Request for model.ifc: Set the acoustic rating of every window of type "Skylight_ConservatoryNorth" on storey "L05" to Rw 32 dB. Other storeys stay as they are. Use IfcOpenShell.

First a look at what the model holds.

```python
import ifcopenshell
import ifcopenshell.util.element

model = ifcopenshell.open("model.ifc")
print(model.schema)
storey = next(s for s in model.by_type("IfcBuildingStorey") if s.Name == "L05")
windows = [e for e in ifcopenshell.util.element.get_decomposition(storey) if e.is_a("IfcWindow")]
seen = {}
for e in windows:
    element_type = ifcopenshell.util.element.get_type(e)
    key = (element_type.Name if element_type != e and element_type else None, ifcopenshell.util.element.get_pset(e, "Pset_WindowCommon", "AcousticRating"))
    seen[key] = seen.get(key, 0) + 1
for (name, value), count in sorted(seen.items(), key=str):
    print(count, "x", name, "|", value)
```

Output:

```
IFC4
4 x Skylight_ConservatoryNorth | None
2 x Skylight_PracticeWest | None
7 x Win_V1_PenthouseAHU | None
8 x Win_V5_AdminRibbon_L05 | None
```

```python
import ifcopenshell
import ifcopenshell.api.pset
import ifcopenshell.util.element

model = ifcopenshell.open("model.ifc")

storey = next(s for s in model.by_type("IfcBuildingStorey") if s.Name == "L05")
windows = [e for e in ifcopenshell.util.element.get_decomposition(storey) if e.is_a("IfcWindow")]

count = 0
for e in windows:
    element_type = ifcopenshell.util.element.get_type(e)
    if element_type in (None, e) or element_type.Name != "Skylight_ConservatoryNorth":
        continue
    # add_pset returns the element's existing set when there is one.
    pset = ifcopenshell.api.pset.add_pset(model, product=e, name="Pset_WindowCommon")
    ifcopenshell.api.pset.edit_pset(model, pset=pset, properties={"AcousticRating": "Rw 32 dB"})
    count += 1

print(count, "windows updated")

model.write("model_edited.ifc")
```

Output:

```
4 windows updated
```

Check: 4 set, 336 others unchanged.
